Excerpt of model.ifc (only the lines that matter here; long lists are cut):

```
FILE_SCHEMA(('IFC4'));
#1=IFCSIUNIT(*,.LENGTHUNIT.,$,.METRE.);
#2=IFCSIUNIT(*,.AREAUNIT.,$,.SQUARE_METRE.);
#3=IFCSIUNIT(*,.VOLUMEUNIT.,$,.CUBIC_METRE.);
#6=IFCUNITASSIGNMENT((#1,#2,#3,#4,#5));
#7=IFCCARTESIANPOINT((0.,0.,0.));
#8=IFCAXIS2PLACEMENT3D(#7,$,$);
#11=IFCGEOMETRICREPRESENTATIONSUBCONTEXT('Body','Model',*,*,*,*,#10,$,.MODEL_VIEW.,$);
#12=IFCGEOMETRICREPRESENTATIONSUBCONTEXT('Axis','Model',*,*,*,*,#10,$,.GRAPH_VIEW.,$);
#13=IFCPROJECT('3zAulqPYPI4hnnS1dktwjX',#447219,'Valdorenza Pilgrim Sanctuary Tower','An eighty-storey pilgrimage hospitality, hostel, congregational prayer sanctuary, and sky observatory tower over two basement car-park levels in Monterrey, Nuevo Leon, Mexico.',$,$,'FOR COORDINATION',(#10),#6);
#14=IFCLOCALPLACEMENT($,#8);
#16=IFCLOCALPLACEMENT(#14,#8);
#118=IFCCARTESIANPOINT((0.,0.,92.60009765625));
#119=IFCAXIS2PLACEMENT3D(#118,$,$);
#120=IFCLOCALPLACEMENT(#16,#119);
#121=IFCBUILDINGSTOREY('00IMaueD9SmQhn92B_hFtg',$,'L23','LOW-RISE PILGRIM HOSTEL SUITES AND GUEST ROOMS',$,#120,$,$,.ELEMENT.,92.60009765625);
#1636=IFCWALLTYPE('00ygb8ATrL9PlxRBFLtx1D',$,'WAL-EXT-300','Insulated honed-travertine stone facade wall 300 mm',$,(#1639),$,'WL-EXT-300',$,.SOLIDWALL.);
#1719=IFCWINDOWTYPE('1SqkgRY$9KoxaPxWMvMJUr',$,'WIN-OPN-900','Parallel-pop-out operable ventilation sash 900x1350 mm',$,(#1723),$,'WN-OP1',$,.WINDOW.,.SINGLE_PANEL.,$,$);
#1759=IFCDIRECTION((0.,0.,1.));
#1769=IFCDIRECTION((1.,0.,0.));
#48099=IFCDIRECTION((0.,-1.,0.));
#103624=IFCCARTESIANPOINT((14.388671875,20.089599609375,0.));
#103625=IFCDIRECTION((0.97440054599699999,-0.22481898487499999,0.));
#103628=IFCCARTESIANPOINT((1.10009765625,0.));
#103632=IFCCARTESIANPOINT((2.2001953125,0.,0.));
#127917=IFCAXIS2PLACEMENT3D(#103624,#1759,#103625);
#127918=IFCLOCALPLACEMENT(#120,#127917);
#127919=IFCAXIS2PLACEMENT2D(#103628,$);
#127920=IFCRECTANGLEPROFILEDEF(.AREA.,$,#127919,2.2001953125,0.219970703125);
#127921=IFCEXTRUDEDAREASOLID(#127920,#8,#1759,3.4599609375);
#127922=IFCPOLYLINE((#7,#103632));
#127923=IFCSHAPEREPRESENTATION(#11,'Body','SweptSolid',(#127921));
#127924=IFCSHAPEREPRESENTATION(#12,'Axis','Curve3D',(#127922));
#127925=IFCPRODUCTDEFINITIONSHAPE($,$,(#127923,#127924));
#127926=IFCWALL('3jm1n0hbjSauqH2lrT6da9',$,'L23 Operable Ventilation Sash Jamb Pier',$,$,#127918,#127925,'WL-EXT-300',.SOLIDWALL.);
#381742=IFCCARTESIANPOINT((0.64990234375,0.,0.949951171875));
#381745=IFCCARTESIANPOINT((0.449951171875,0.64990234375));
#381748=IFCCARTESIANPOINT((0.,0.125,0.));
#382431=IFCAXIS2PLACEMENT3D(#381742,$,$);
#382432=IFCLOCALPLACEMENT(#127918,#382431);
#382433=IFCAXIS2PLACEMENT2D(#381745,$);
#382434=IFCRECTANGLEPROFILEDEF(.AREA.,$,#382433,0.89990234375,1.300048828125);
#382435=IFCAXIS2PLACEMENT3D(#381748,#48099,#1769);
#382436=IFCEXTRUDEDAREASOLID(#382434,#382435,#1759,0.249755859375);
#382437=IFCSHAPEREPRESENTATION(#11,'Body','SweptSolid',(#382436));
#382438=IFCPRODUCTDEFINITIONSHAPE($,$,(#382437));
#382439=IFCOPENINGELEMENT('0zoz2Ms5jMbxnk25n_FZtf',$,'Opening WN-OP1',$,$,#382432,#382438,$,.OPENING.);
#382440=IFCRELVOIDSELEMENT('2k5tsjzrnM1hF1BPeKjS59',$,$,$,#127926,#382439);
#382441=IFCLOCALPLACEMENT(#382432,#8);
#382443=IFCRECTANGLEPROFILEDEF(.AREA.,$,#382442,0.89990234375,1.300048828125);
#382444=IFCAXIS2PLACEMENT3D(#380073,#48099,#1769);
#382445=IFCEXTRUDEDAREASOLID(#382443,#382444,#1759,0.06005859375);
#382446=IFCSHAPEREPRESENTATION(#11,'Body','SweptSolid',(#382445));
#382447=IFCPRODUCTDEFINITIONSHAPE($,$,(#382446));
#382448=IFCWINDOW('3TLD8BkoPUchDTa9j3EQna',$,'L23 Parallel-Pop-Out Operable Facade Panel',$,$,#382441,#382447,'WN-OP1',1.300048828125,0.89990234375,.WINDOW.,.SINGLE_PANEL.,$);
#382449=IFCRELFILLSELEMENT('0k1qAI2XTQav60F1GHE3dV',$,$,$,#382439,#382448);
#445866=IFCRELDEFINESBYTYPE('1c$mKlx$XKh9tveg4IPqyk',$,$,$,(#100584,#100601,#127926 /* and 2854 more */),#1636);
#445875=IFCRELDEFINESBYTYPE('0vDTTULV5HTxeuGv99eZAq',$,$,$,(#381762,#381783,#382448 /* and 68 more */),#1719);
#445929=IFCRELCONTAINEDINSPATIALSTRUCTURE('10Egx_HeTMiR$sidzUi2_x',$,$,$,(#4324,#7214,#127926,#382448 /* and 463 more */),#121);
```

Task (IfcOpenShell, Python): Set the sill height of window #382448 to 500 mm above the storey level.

```python
import numpy as np
import ifcopenshell
import ifcopenshell.api.geometry
import ifcopenshell.geom
import ifcopenshell.util.element
import ifcopenshell.util.placement
import ifcopenshell.util.shape
import ifcopenshell.util.unit

model = ifcopenshell.open("model.ifc")
unit_scale = ifcopenshell.util.unit.calculate_unit_scale(model)

window = model.by_guid("3TLD8BkoPUchDTa9j3EQna")
opening = window.FillsVoids[0].RelatingOpeningElement
storey = ifcopenshell.util.element.get_container(window, ifc_class="IfcBuildingStorey")
level = ifcopenshell.util.placement.get_local_placement(storey.ObjectPlacement)[2, 3]

# The opening's origin need not be at the sill, so measure its lowest point.
shape = ifcopenshell.geom.create_shape(ifcopenshell.geom.settings(), opening)
bottom = ifcopenshell.util.shape.get_shape_bottom_elevation(shape, shape.geometry) / unit_scale
dz = level + 0.5 - bottom

shift = np.array([0.0, 0.0, dz])
# The window is placed relative to its opening, so it follows when the opening moves.
matrix = ifcopenshell.util.placement.get_local_placement(opening.ObjectPlacement)
matrix[:3, 3] += shift
ifcopenshell.api.geometry.edit_object_placement(
    model, product=opening, matrix=matrix, is_si=False, should_transform_children=True
)

print(f"moved by {dz * unit_scale:+.3f} m")

model.write("model_v2.ifc")
```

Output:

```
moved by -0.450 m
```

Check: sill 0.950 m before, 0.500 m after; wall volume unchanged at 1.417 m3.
